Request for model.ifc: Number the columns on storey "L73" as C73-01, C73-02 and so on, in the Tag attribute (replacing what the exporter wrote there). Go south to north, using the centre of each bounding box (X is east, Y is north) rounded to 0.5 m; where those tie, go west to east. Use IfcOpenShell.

First a look at what the model holds.

```python
import ifcopenshell
import ifcopenshell.util.element
import ifcopenshell.util.placement

model = ifcopenshell.open("model.ifc")
print(model.schema)
storey = next(s for s in model.by_type("IfcBuildingStorey") if s.Name == "L73")
columns = [e for e in ifcopenshell.util.element.get_decomposition(storey) if e.is_a("IfcColumn")]
for e in sorted(columns, key=lambda e: e.id()):
    origin = ifcopenshell.util.placement.get_local_placement(e.ObjectPlacement)[:3, 3]
    print(e.id(), e.Tag, e.Name, origin.round(2) + 0.0, sep=" | ")
```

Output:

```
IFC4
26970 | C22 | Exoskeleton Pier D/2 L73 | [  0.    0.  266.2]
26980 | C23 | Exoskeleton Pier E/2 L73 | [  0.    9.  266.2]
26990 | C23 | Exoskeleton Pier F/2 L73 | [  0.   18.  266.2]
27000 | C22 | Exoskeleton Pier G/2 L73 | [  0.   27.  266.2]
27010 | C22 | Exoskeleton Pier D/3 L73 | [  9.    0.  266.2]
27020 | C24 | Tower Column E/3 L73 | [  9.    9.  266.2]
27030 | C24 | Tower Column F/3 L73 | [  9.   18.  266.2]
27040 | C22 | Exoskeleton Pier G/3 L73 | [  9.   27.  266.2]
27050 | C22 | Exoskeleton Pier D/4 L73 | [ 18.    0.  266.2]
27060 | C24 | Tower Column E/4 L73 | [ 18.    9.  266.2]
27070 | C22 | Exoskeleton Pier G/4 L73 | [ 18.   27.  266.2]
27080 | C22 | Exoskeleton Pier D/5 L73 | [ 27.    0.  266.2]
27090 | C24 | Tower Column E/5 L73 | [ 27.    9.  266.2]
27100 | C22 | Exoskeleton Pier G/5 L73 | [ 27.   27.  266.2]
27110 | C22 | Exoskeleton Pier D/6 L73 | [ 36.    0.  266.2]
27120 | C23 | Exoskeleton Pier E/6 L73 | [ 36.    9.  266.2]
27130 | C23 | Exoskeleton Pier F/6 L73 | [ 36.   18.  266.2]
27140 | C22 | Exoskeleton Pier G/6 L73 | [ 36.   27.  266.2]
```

```python
import ifcopenshell
import ifcopenshell.geom
import ifcopenshell.util.element
import ifcopenshell.util.shape

model = ifcopenshell.open("model.ifc")
settings = ifcopenshell.geom.settings()
settings.set("use-world-coords", True)


def centre(element):
    shape = ifcopenshell.geom.create_shape(settings, element)
    return ifcopenshell.util.shape.get_bbox_centroid(shape.geometry)


storey = next(s for s in model.by_type("IfcBuildingStorey") if s.Name == "L73")
columns = [e for e in ifcopenshell.util.element.get_decomposition(storey) if e.is_a("IfcColumn")]

# Insertion points can sit at a corner or the storey origin, so sort by the geometry (in metres).
centres = {e: centre(e) for e in columns}
columns.sort(key=lambda e: (round(centres[e][1] / 0.5), centres[e][0]))

for i, e in enumerate(columns, start=1):
    number = f"C73-{i:02d}"
    e.Tag = number
    print(e.id(), number)

model.write("model_rev.ifc")
```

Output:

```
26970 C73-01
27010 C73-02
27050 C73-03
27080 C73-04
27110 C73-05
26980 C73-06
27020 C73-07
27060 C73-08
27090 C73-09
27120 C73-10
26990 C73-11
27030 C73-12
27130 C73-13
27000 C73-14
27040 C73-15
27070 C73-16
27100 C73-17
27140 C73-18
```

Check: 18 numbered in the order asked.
